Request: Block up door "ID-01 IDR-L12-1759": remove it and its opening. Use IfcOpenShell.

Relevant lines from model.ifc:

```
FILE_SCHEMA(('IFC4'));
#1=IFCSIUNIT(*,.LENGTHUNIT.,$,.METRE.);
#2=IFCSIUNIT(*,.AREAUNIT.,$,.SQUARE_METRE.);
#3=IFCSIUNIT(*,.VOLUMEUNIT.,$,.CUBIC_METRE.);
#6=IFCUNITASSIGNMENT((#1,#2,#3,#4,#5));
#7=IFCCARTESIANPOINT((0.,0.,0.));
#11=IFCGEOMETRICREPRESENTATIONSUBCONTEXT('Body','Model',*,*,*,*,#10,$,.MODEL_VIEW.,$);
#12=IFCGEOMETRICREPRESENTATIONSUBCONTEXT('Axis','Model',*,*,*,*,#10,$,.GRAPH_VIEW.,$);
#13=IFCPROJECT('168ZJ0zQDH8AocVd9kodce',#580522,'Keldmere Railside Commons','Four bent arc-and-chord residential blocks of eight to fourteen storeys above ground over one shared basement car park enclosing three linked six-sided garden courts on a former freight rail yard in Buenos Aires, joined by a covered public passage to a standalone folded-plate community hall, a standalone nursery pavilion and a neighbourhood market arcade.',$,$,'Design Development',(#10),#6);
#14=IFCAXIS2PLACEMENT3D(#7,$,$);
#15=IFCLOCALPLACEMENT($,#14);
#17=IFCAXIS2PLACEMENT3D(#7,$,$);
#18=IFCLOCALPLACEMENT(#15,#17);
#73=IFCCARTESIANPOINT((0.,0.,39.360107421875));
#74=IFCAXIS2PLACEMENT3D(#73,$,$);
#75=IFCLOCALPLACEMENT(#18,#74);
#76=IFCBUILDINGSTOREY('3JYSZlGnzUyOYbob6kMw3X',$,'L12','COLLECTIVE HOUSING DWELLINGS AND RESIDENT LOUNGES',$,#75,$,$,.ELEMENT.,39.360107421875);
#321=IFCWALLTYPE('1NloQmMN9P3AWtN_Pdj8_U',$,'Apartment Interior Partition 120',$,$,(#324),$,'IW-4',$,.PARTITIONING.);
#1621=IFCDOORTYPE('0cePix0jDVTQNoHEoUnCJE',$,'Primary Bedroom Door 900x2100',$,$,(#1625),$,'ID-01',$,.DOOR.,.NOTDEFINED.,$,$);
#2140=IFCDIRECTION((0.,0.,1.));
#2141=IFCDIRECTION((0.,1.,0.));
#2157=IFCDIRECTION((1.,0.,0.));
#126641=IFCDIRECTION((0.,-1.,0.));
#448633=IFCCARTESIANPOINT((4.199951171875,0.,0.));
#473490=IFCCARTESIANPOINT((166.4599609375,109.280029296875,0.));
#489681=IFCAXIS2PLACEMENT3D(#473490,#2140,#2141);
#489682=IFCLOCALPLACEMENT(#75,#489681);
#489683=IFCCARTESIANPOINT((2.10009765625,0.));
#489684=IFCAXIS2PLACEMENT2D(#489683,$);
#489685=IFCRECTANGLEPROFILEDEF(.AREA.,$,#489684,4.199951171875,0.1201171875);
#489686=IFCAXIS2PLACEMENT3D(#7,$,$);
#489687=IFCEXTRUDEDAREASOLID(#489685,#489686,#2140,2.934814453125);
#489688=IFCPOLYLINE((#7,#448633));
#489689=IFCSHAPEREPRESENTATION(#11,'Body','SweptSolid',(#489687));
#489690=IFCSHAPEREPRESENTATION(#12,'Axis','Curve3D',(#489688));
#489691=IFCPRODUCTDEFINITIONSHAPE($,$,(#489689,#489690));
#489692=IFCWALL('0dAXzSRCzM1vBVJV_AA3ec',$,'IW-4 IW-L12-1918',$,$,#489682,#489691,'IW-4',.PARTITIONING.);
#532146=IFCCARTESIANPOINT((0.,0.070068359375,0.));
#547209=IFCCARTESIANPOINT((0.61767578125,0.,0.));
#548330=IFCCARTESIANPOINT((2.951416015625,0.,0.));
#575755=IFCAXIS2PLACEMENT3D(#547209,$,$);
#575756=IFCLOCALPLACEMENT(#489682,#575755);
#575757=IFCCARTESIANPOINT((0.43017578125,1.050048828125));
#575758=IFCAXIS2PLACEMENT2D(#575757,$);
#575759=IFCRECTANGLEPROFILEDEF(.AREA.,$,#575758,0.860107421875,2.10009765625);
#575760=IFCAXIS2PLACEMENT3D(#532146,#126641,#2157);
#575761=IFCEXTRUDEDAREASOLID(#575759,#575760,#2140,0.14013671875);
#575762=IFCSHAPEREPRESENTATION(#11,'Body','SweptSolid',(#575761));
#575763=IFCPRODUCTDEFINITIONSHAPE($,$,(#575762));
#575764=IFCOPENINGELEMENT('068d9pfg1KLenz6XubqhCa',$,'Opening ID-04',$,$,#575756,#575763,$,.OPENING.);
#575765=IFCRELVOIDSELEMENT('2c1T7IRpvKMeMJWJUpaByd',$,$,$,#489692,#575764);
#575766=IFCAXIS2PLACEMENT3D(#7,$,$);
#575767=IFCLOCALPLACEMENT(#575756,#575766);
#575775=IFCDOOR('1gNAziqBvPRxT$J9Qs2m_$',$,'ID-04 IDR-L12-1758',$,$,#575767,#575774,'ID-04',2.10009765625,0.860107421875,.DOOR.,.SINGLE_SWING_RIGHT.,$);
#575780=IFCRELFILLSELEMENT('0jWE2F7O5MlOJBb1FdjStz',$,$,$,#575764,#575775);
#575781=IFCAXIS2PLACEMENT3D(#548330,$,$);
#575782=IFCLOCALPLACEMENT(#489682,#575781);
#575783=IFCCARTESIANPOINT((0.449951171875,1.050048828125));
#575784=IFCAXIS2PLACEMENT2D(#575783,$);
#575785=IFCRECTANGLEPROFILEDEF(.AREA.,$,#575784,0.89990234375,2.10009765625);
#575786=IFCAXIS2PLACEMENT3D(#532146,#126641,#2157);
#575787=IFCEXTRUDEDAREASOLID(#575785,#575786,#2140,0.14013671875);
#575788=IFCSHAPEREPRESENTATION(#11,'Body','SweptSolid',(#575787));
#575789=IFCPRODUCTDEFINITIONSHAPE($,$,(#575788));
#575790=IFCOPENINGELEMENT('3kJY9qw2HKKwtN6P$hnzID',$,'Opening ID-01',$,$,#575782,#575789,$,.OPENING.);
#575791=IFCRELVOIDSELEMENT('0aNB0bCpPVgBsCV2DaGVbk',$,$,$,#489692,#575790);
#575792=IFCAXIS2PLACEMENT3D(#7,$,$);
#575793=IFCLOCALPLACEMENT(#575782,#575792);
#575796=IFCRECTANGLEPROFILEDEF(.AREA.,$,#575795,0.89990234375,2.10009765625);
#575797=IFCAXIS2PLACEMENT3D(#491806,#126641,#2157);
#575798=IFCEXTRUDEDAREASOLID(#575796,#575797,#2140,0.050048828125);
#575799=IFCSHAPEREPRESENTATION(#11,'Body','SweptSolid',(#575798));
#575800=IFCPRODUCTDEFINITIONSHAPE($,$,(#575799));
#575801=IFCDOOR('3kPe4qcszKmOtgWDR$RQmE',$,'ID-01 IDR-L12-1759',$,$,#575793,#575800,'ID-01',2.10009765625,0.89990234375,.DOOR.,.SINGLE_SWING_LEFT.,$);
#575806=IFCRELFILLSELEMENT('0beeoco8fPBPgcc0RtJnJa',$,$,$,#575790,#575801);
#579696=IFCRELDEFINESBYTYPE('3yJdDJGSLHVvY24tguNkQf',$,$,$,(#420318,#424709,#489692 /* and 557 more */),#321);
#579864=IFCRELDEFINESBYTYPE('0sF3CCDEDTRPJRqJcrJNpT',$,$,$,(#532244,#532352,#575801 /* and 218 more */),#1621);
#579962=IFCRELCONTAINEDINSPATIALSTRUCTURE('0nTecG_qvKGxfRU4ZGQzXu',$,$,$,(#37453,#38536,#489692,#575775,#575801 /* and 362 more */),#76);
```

```python
import ifcopenshell
import ifcopenshell.api.feature
import ifcopenshell.api.root
import ifcopenshell.geom
import ifcopenshell.util.shape

model = ifcopenshell.open("model.ifc")
settings = ifcopenshell.geom.settings()


def volume(element):
    """Net volume in cubic metres, openings subtracted."""
    shape = ifcopenshell.geom.create_shape(settings, element)
    return ifcopenshell.util.shape.get_volume(shape.geometry)


door = model.by_guid("3kPe4qcszKmOtgWDR$RQmE")
opening = door.FillsVoids[0].RelatingOpeningElement
wall = opening.VoidsElements[0].RelatingBuildingElement
before = volume(wall)

ifcopenshell.api.root.remove_product(model, product=door)
ifcopenshell.api.feature.remove_feature(model, feature=opening)

after = volume(wall)

print(f"wall volume {before:.3f} -> {after:.3f} m3")

model.write("model_edited.ifc")
```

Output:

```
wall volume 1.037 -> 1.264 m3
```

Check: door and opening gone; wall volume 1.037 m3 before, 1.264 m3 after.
